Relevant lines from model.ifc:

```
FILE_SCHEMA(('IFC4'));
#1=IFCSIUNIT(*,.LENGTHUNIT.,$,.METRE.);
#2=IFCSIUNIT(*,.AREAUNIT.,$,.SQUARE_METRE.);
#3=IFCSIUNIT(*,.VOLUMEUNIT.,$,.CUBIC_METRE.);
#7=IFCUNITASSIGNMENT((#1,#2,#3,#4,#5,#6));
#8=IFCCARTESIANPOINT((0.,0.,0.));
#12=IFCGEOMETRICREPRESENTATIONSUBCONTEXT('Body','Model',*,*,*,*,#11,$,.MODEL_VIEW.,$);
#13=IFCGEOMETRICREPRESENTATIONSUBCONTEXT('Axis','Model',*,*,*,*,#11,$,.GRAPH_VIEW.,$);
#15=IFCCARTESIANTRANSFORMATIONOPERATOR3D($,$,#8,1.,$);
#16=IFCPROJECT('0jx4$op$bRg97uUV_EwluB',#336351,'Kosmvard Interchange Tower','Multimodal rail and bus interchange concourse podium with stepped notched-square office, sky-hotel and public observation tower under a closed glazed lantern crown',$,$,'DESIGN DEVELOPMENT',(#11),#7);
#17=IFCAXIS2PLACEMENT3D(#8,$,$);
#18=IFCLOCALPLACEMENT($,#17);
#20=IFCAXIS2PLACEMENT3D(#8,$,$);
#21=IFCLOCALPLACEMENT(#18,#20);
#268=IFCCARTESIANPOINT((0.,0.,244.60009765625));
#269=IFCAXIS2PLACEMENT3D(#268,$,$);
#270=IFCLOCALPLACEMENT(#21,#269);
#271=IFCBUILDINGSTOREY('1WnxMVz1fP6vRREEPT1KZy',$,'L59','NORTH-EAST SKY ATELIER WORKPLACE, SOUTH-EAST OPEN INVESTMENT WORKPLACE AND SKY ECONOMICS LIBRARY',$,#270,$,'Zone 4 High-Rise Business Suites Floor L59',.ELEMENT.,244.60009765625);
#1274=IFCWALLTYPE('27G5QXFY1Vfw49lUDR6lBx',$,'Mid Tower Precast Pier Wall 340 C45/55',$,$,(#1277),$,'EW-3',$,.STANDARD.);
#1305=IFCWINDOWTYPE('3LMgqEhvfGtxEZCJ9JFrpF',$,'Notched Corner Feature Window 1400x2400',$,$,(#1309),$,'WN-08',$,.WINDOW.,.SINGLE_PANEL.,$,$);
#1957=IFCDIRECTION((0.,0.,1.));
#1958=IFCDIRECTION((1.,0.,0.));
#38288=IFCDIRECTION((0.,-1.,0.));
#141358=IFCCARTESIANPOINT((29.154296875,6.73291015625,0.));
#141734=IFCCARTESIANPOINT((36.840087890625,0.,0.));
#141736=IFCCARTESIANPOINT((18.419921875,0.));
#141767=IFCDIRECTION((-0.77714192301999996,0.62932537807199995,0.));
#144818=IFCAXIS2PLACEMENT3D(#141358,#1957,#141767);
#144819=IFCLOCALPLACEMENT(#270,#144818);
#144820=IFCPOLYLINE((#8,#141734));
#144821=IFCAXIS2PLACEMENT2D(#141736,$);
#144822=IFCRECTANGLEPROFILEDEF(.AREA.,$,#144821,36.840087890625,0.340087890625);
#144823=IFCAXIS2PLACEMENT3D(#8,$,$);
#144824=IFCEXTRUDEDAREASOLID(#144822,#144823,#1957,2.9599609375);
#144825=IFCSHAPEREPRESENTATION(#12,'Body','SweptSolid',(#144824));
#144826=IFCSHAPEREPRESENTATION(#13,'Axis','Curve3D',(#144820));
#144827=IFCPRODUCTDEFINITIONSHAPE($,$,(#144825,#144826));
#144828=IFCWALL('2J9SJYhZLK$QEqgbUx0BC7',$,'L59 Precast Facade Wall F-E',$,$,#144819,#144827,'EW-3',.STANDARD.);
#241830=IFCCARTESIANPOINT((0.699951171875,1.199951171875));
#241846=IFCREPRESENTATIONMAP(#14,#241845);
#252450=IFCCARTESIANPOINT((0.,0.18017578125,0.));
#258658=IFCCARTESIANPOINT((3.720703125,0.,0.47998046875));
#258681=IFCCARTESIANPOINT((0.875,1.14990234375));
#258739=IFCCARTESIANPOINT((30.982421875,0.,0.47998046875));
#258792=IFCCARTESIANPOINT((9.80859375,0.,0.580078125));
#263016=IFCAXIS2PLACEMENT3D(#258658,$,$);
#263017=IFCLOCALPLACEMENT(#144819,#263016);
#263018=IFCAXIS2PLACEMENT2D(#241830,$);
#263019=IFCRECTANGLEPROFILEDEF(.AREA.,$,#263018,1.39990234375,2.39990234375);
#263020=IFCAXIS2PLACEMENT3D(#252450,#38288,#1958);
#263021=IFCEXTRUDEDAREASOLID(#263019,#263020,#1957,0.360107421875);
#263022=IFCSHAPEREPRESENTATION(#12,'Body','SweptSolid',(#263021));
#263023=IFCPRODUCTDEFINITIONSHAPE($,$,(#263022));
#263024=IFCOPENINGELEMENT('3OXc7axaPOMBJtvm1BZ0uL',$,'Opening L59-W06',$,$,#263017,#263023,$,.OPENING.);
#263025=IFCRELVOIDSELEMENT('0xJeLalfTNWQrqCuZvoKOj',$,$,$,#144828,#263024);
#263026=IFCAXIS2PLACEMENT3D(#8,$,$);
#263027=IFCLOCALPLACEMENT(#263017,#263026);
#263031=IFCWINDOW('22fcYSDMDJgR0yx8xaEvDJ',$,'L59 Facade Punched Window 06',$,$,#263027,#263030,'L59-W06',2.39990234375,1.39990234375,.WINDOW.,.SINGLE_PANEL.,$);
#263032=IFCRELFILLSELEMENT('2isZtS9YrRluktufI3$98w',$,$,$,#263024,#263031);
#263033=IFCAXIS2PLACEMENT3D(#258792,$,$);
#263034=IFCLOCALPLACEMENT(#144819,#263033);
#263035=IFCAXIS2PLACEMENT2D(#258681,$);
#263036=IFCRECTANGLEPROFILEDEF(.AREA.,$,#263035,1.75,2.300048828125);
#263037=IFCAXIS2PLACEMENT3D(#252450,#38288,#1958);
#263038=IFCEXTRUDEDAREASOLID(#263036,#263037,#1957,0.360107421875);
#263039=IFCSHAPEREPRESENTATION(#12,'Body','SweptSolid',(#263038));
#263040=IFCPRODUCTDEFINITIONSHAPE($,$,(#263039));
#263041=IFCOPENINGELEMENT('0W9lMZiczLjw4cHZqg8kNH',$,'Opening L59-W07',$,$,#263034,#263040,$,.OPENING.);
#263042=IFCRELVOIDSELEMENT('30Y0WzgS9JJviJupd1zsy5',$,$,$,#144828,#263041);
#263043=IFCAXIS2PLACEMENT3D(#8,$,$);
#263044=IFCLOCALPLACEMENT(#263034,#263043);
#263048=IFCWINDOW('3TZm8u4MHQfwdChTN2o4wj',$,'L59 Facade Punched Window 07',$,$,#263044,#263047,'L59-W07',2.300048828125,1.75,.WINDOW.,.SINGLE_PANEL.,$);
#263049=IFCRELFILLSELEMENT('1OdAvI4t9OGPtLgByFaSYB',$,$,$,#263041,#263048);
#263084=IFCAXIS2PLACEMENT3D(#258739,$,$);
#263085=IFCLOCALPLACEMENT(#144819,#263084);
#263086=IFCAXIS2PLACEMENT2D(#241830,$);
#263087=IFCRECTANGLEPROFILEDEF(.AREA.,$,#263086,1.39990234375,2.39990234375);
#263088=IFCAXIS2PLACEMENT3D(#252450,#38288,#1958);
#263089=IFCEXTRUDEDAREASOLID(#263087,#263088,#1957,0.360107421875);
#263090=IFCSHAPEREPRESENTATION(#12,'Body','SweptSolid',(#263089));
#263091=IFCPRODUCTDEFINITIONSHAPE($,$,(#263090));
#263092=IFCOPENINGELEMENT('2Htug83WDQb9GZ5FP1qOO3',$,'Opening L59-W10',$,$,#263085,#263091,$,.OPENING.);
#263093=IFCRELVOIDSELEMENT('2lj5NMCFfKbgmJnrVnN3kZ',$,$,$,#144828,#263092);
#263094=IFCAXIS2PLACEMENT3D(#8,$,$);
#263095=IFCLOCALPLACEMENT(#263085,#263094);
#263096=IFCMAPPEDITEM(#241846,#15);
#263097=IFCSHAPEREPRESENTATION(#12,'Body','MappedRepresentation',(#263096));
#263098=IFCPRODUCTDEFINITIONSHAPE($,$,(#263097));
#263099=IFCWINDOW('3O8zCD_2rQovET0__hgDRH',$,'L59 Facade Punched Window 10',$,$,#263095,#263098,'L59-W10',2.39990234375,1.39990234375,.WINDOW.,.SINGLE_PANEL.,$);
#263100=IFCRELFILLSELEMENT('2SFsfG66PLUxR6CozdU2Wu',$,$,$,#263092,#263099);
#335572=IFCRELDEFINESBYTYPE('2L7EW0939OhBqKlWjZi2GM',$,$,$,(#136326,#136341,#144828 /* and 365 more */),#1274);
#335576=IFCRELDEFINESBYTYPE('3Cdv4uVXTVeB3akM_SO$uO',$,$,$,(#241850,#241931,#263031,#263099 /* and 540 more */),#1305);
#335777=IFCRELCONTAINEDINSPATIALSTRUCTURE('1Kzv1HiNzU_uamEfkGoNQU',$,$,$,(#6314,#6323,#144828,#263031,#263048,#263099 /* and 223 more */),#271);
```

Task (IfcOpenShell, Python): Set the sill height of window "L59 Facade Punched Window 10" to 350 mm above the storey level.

```python
import numpy as np
import ifcopenshell
import ifcopenshell.api.geometry
import ifcopenshell.geom
import ifcopenshell.util.element
import ifcopenshell.util.placement
import ifcopenshell.util.shape
import ifcopenshell.util.unit

model = ifcopenshell.open("model.ifc")
unit_scale = ifcopenshell.util.unit.calculate_unit_scale(model)

window = model.by_guid("3O8zCD_2rQovET0__hgDRH")
opening = window.FillsVoids[0].RelatingOpeningElement
storey = ifcopenshell.util.element.get_container(window, ifc_class="IfcBuildingStorey")
level = ifcopenshell.util.placement.get_local_placement(storey.ObjectPlacement)[2, 3]

# The opening's origin need not be at the sill, so measure its lowest point.
shape = ifcopenshell.geom.create_shape(ifcopenshell.geom.settings(), opening)
bottom = ifcopenshell.util.shape.get_shape_bottom_elevation(shape, shape.geometry) / unit_scale
dz = level + 0.35 - bottom

shift = np.array([0.0, 0.0, dz])
# The window is placed relative to its opening, so it follows when the opening moves.
matrix = ifcopenshell.util.placement.get_local_placement(opening.ObjectPlacement)
matrix[:3, 3] += shift
ifcopenshell.api.geometry.edit_object_placement(
    model, product=opening, matrix=matrix, is_si=False, should_transform_children=True
)

print(f"moved by {dz * unit_scale:+.3f} m")

model.write("model_v2.ifc")
```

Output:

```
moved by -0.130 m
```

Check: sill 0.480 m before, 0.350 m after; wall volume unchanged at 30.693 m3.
